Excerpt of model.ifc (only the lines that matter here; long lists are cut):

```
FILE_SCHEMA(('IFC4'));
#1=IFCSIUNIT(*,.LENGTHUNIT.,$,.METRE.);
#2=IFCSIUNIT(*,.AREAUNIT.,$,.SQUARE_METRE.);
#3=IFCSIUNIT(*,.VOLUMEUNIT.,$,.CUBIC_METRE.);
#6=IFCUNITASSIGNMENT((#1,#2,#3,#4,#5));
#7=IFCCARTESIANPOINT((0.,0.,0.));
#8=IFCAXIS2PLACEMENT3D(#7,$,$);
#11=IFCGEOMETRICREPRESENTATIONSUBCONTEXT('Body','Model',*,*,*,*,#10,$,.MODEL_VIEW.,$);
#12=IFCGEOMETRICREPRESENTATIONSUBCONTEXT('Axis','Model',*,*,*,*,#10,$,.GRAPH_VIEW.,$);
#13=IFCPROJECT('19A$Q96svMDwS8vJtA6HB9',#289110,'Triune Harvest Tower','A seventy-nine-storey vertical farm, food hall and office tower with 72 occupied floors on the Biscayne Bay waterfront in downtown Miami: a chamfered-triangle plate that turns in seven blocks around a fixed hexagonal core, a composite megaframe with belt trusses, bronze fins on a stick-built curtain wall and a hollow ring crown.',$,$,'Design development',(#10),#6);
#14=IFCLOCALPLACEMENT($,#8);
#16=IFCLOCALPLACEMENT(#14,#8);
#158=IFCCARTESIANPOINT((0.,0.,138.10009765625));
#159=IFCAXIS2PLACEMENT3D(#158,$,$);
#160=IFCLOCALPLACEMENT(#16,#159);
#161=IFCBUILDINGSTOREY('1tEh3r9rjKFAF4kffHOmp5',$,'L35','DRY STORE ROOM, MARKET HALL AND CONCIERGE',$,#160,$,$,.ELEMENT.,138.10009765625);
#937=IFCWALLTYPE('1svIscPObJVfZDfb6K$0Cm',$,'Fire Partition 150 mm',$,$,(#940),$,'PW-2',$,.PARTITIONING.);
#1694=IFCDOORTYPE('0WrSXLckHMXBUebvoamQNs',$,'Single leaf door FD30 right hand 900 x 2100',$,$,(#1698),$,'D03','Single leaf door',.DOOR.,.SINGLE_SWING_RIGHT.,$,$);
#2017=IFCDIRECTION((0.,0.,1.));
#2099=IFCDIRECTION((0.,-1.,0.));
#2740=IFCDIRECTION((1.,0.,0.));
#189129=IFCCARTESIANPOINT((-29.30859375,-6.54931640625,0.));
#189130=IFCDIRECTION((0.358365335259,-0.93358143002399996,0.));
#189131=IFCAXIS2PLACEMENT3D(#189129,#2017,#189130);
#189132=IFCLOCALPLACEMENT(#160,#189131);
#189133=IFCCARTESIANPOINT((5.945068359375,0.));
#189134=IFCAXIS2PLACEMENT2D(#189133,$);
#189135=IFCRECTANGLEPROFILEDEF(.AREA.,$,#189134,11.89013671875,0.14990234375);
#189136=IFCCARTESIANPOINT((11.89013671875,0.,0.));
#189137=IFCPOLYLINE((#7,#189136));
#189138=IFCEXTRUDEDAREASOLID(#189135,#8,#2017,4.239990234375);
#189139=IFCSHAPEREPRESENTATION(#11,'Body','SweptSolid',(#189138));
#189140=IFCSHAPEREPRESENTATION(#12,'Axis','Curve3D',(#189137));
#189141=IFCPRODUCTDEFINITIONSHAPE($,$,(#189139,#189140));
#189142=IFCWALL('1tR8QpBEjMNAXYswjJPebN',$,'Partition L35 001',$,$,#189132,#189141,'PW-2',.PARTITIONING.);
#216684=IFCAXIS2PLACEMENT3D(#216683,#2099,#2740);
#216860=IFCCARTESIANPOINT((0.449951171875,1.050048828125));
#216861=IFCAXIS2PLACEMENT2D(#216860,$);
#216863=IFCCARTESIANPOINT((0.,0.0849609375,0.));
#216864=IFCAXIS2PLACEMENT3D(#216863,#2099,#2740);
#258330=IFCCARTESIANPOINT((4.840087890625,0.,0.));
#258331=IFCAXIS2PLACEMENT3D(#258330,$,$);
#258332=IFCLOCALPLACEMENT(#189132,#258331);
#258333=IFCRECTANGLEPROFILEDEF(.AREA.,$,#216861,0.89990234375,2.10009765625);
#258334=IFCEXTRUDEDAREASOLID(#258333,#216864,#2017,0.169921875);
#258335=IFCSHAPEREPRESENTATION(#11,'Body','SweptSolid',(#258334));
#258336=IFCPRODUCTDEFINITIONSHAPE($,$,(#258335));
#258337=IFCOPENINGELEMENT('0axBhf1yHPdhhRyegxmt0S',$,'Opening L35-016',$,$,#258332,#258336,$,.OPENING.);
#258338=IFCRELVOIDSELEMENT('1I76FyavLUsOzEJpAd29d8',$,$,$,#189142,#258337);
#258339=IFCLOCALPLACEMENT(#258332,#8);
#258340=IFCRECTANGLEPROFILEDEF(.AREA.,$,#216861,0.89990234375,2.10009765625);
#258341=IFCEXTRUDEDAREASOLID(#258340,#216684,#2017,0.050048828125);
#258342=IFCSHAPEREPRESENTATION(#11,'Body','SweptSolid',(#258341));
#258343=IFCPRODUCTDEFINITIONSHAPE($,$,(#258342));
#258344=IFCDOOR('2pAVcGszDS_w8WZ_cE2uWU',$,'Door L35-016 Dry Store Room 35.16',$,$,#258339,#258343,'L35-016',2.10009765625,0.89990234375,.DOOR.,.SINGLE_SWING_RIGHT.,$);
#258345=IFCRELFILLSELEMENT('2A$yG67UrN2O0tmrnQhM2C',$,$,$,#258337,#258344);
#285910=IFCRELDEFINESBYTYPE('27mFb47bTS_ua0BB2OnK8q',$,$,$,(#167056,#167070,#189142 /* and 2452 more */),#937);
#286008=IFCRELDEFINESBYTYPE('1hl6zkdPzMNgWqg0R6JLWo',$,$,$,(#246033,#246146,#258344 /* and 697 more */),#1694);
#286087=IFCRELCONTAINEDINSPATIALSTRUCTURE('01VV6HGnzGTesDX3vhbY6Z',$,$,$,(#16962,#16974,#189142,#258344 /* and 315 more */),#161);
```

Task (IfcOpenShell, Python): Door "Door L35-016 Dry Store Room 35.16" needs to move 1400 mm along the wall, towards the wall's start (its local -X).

```python
import ifcopenshell
import ifcopenshell.api.geometry
import ifcopenshell.util.placement

model = ifcopenshell.open("model.ifc")

door = model.by_guid("2pAVcGszDS_w8WZ_cE2uWU")
opening = door.FillsVoids[0].RelatingOpeningElement
wall = opening.VoidsElements[0].RelatingBuildingElement

wall_matrix = ifcopenshell.util.placement.get_local_placement(wall.ObjectPlacement)
shift = wall_matrix[:3, 0] * -1.4
before = ifcopenshell.util.placement.get_local_placement(door.ObjectPlacement)[:3, 3].copy()

# The door is placed relative to its opening, so it follows when the opening moves.
matrix = ifcopenshell.util.placement.get_local_placement(opening.ObjectPlacement)
matrix[:3, 3] += shift
ifcopenshell.api.geometry.edit_object_placement(
    model, product=opening, matrix=matrix, is_si=False, should_transform_children=True
)

after = ifcopenshell.util.placement.get_local_placement(door.ObjectPlacement)[:3, 3]
print("door moved by", (after - before).round(3) + 0.0)

model.write("model_updated.ifc")
```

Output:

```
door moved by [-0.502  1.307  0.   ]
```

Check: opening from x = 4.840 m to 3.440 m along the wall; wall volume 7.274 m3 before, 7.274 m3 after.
